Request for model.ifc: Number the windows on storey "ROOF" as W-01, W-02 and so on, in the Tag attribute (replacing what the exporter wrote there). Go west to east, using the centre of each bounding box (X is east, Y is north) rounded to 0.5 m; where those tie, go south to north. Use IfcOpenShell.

First a look at what the model holds.

```python
import ifcopenshell
import ifcopenshell.util.element
import ifcopenshell.util.placement

model = ifcopenshell.open("model.ifc")
print(model.schema)
storey = next(s for s in model.by_type("IfcBuildingStorey") if s.Name == "ROOF")
windows = [e for e in ifcopenshell.util.element.get_decomposition(storey) if e.is_a("IfcWindow")]
for e in sorted(windows, key=lambda e: e.id()):
    origin = ifcopenshell.util.placement.get_local_placement(e.ObjectPlacement)[:3, 3]
    print(e.id(), e.Tag, e.Name, origin.round(2) + 0.0, sep=" | ")
```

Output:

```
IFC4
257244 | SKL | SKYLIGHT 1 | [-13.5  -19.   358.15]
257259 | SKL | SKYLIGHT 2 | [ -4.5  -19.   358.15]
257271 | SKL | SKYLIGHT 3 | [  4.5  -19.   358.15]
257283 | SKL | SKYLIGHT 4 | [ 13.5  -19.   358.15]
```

```python
import ifcopenshell
import ifcopenshell.geom
import ifcopenshell.util.element
import ifcopenshell.util.shape

model = ifcopenshell.open("model.ifc")
settings = ifcopenshell.geom.settings()
settings.set("use-world-coords", True)


def centre(element):
    shape = ifcopenshell.geom.create_shape(settings, element)
    return ifcopenshell.util.shape.get_bbox_centroid(shape.geometry)


storey = next(s for s in model.by_type("IfcBuildingStorey") if s.Name == "ROOF")
windows = [e for e in ifcopenshell.util.element.get_decomposition(storey) if e.is_a("IfcWindow")]

# Insertion points can sit at a corner or the storey origin, so sort by the geometry (in metres).
centres = {e: centre(e) for e in windows}
windows.sort(key=lambda e: (round(centres[e][0] / 0.5), centres[e][1]))

for i, e in enumerate(windows, start=1):
    number = f"W-{i:02d}"
    e.Tag = number
    print(e.id(), number)

model.write("model_edited.ifc")
```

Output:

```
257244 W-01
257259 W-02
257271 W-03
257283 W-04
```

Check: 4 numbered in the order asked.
